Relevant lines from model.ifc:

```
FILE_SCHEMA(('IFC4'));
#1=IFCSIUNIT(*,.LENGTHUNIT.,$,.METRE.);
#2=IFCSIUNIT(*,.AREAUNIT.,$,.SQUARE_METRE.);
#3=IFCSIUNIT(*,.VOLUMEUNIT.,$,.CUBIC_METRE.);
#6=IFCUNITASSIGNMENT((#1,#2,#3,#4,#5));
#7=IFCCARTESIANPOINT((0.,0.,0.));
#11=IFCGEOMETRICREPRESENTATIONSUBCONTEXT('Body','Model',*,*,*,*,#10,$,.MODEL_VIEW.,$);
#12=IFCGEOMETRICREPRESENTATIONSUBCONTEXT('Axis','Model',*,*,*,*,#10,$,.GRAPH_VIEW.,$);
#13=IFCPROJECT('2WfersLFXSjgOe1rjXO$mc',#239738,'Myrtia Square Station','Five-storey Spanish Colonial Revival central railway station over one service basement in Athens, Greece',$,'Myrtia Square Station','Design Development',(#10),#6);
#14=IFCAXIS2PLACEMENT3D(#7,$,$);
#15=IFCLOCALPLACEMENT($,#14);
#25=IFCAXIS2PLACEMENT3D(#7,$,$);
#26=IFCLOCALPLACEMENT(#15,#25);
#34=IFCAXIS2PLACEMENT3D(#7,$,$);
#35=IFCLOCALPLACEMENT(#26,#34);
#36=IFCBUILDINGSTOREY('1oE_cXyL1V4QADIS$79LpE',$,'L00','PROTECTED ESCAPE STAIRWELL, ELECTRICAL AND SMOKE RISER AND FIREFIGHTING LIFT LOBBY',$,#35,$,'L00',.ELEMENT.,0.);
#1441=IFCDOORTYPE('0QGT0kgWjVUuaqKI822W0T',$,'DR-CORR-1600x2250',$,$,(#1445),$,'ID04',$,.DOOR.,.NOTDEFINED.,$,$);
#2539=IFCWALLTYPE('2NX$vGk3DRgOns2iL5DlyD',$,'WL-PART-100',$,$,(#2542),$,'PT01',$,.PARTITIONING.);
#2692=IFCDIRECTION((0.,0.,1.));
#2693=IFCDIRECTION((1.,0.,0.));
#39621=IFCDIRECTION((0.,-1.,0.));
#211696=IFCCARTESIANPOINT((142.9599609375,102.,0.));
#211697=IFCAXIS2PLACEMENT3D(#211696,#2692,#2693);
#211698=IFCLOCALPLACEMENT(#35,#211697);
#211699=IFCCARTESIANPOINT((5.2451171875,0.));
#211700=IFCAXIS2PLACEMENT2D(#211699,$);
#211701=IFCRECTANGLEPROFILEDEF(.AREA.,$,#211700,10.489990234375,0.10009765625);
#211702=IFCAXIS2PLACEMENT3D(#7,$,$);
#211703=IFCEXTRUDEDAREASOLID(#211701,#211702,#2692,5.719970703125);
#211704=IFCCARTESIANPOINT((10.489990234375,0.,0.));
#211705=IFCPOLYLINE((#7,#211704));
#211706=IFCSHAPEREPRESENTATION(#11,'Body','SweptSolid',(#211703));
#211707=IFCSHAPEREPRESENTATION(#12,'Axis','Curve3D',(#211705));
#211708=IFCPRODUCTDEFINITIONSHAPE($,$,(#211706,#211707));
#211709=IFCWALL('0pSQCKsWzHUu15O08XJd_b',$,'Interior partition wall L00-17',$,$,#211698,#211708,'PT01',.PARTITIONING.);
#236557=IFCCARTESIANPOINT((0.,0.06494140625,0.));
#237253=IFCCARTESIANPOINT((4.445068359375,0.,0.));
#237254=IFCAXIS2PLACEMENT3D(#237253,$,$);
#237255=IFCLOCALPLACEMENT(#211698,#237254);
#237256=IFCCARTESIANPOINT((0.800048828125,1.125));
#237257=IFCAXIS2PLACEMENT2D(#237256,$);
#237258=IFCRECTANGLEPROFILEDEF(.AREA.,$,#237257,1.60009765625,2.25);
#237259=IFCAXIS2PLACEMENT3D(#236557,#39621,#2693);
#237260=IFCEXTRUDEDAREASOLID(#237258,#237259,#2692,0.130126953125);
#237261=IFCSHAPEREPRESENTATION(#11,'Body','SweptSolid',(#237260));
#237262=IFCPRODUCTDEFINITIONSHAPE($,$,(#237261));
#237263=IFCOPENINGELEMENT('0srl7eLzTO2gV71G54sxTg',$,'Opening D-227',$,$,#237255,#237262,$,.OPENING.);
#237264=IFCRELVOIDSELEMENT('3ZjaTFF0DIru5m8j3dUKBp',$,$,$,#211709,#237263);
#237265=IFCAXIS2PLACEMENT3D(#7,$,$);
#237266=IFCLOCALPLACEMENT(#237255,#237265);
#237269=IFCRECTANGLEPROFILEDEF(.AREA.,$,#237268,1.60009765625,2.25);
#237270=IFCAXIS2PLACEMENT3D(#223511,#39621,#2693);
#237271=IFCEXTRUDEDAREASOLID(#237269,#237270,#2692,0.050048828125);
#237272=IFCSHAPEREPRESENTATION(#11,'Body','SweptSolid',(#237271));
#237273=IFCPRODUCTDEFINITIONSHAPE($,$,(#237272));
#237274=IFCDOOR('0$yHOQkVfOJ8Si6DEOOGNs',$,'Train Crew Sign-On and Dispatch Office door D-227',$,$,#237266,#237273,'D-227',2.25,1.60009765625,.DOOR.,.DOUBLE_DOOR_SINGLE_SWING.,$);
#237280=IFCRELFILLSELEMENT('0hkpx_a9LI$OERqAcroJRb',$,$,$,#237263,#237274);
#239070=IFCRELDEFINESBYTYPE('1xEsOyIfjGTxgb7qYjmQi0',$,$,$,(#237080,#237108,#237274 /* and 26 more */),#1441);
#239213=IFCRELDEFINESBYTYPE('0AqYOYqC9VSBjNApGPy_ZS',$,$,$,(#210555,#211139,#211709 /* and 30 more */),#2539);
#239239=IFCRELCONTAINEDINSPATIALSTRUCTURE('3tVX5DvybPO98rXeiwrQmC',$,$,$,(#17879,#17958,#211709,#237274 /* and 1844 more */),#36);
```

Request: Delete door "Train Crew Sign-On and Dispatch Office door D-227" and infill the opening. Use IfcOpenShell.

```python
import ifcopenshell
import ifcopenshell.api.feature
import ifcopenshell.api.root
import ifcopenshell.geom
import ifcopenshell.util.shape

model = ifcopenshell.open("model.ifc")
settings = ifcopenshell.geom.settings()


def volume(element):
    """Net volume in cubic metres, openings subtracted."""
    shape = ifcopenshell.geom.create_shape(settings, element)
    return ifcopenshell.util.shape.get_volume(shape.geometry)


door = model.by_id(237274)
opening = door.FillsVoids[0].RelatingOpeningElement
wall = opening.VoidsElements[0].RelatingBuildingElement
before = volume(wall)

ifcopenshell.api.root.remove_product(model, product=door)
ifcopenshell.api.feature.remove_feature(model, feature=opening)

after = volume(wall)

print(f"wall volume {before:.3f} -> {after:.3f} m3")

model.write("model_edited.ifc")
```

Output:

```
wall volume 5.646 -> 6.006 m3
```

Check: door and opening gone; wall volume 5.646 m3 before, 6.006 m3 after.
